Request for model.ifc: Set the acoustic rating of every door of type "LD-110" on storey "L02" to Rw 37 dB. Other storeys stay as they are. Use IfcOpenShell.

First a look at what the model holds.

```python
import ifcopenshell
import ifcopenshell.util.element

model = ifcopenshell.open("model.ifc")
print(model.schema)
storey = next(s for s in model.by_type("IfcBuildingStorey") if s.Name == "L02")
doors = [e for e in ifcopenshell.util.element.get_decomposition(storey) if e.is_a("IfcDoor")]
seen = {}
for e in doors:
    element_type = ifcopenshell.util.element.get_type(e)
    key = (element_type.Name if element_type != e and element_type else None, ifcopenshell.util.element.get_pset(e, "Pset_DoorCommon", "AcousticRating"))
    seen[key] = seen.get(key, 0) + 1
for (name, value), count in sorted(seen.items(), key=str):
    print(count, "x", name, "|", value)
```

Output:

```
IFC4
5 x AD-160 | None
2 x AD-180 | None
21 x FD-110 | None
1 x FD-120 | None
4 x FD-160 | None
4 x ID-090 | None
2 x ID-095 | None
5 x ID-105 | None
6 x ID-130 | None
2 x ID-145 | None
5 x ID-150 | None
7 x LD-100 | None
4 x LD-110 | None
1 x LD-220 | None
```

```python
import ifcopenshell
import ifcopenshell.api.pset
import ifcopenshell.util.element

model = ifcopenshell.open("model.ifc")

storey = next(s for s in model.by_type("IfcBuildingStorey") if s.Name == "L02")
doors = [e for e in ifcopenshell.util.element.get_decomposition(storey) if e.is_a("IfcDoor")]

count = 0
for e in doors:
    element_type = ifcopenshell.util.element.get_type(e)
    if element_type in (None, e) or element_type.Name != "LD-110":
        continue
    # add_pset returns the element's existing set when there is one.
    pset = ifcopenshell.api.pset.add_pset(model, product=e, name="Pset_DoorCommon")
    ifcopenshell.api.pset.edit_pset(model, pset=pset, properties={"AcousticRating": "Rw 37 dB"})
    count += 1

print(count, "doors updated")

model.write("model_edited.ifc")
```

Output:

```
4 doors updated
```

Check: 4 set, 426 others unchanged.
